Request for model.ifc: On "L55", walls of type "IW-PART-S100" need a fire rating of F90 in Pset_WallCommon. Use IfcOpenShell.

First a look at what the model holds.

```python
import ifcopenshell
import ifcopenshell.util.element

model = ifcopenshell.open("model.ifc")
print(model.schema)
storey = next(s for s in model.by_type("IfcBuildingStorey") if s.Name == "L55")
walls = [e for e in ifcopenshell.util.element.get_decomposition(storey) if e.is_a("IfcWall")]
seen = {}
for e in walls:
    element_type = ifcopenshell.util.element.get_type(e)
    key = (element_type.Name if element_type != e and element_type else None, ifcopenshell.util.element.get_pset(e, "Pset_WallCommon", "FireRating"))
    seen[key] = seen.get(key, 0) + 1
for (name, value), count in sorted(seen.items(), key=str):
    print(count, "x", name, "|", value)
```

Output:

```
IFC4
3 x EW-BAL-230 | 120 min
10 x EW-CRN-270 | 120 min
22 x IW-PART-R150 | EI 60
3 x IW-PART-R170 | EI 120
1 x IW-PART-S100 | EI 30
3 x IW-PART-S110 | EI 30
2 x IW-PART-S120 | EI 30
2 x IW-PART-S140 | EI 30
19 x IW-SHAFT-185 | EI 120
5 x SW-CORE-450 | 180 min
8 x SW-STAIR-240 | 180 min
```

```python
import ifcopenshell
import ifcopenshell.api.pset
import ifcopenshell.util.element

model = ifcopenshell.open("model.ifc")

storey = next(s for s in model.by_type("IfcBuildingStorey") if s.Name == "L55")
walls = [e for e in ifcopenshell.util.element.get_decomposition(storey) if e.is_a("IfcWall")]

count = 0
for e in walls:
    element_type = ifcopenshell.util.element.get_type(e)
    if element_type in (None, e) or element_type.Name != "IW-PART-S100":
        continue
    # add_pset returns the element's existing set when there is one.
    pset = ifcopenshell.api.pset.add_pset(model, product=e, name="Pset_WallCommon")
    ifcopenshell.api.pset.edit_pset(model, pset=pset, properties={"FireRating": "F90"})
    count += 1

print(count, "walls updated")

model.write("model_updated.ifc")
```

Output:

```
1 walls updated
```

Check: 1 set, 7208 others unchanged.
